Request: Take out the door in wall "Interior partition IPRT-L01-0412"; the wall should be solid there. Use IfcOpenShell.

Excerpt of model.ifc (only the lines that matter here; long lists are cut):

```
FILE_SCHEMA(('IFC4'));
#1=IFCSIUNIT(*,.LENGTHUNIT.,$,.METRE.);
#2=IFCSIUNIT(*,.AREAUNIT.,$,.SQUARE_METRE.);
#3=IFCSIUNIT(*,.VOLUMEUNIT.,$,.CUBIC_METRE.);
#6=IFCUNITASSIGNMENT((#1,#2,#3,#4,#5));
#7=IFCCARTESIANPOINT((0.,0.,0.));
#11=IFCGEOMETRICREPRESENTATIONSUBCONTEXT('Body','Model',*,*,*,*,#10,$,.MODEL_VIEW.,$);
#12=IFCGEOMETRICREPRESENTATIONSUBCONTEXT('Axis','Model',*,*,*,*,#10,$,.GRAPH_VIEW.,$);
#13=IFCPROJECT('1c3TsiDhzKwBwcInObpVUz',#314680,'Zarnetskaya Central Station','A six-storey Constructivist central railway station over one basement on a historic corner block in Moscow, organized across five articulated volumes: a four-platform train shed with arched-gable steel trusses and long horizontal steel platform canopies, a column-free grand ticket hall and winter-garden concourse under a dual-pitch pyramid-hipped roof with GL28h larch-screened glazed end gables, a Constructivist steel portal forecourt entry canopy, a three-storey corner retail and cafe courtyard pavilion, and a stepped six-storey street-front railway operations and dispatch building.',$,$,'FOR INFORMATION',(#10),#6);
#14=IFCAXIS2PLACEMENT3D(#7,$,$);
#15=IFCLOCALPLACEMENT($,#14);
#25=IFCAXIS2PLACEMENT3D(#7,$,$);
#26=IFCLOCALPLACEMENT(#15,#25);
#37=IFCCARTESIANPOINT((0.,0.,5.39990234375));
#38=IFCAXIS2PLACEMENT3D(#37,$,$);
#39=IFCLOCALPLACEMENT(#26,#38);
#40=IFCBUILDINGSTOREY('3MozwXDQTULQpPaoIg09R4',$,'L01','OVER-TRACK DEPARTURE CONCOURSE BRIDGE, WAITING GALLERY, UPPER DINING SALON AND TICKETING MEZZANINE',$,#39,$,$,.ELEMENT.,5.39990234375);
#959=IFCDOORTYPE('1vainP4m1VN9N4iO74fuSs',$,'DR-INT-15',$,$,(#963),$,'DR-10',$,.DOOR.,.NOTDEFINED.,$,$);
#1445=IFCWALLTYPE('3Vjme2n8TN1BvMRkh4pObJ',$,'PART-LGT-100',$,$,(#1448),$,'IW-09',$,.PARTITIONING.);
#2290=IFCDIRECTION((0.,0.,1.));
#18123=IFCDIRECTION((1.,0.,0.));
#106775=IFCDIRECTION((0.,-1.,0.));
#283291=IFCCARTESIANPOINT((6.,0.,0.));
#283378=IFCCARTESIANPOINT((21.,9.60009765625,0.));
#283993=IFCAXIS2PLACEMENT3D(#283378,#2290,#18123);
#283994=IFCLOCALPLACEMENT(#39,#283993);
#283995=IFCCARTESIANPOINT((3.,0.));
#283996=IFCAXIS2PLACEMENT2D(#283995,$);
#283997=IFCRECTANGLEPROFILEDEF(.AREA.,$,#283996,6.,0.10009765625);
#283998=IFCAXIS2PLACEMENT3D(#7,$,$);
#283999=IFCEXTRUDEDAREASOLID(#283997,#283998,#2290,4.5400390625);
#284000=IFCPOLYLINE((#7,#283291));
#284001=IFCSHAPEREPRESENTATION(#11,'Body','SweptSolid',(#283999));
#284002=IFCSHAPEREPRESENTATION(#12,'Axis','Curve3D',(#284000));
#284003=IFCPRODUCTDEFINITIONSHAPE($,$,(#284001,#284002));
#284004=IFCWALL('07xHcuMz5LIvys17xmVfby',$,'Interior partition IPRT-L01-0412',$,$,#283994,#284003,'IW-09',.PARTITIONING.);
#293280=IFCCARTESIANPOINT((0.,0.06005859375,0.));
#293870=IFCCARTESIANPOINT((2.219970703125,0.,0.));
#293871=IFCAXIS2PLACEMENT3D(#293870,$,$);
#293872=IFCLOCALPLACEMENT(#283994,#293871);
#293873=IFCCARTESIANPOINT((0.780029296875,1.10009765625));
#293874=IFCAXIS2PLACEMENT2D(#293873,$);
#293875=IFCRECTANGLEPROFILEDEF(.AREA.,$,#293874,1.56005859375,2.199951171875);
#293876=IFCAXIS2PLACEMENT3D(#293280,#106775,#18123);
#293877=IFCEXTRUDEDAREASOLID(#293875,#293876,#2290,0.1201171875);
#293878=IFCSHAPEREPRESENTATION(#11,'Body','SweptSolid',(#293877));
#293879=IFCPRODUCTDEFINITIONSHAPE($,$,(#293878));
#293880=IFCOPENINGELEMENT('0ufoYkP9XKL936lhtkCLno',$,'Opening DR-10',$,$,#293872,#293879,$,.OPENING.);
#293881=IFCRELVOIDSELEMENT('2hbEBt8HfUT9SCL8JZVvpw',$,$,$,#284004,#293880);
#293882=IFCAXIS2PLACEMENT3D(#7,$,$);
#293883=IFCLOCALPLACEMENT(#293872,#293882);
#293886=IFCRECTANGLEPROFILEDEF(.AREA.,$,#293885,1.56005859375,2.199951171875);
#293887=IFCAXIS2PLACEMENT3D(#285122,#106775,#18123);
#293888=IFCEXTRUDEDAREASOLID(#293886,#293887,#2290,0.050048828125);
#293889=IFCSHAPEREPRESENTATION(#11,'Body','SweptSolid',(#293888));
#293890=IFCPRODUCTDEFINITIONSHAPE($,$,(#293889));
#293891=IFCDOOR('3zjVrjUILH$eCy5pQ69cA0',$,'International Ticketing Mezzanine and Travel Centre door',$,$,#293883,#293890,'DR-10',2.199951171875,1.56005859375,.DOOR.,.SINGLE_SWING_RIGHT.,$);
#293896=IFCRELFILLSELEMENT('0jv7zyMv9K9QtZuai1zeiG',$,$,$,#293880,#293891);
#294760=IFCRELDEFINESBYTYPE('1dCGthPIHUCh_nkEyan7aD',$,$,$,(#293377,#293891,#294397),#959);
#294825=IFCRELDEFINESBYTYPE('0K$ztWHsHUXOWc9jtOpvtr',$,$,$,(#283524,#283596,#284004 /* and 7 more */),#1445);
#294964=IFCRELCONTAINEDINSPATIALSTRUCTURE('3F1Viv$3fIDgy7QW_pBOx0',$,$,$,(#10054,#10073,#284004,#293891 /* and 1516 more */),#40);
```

```python
import ifcopenshell
import ifcopenshell.api.feature
import ifcopenshell.api.root
import ifcopenshell.geom
import ifcopenshell.util.shape

model = ifcopenshell.open("model.ifc")
settings = ifcopenshell.geom.settings()


def volume(element):
    """Net volume in cubic metres, openings subtracted."""
    shape = ifcopenshell.geom.create_shape(settings, element)
    return ifcopenshell.util.shape.get_volume(shape.geometry)


door = model.by_guid("3zjVrjUILH$eCy5pQ69cA0")
opening = door.FillsVoids[0].RelatingOpeningElement
wall = opening.VoidsElements[0].RelatingBuildingElement
before = volume(wall)

ifcopenshell.api.root.remove_product(model, product=door)
ifcopenshell.api.feature.remove_feature(model, feature=opening)

after = volume(wall)

print(f"wall volume {before:.3f} -> {after:.3f} m3")

model.write("model_rev.ifc")
```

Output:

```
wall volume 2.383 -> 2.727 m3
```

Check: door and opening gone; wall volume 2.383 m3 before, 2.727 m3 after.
